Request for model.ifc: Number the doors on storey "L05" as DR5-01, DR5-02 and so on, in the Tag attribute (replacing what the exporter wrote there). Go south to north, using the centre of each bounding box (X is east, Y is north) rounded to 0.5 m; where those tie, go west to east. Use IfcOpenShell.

First a look at what the model holds.

```python
import ifcopenshell
import ifcopenshell.util.element
import ifcopenshell.util.placement

model = ifcopenshell.open("model.ifc")
print(model.schema)
storey = next(s for s in model.by_type("IfcBuildingStorey") if s.Name == "L05")
doors = [e for e in ifcopenshell.util.element.get_decomposition(storey) if e.is_a("IfcDoor")]
for e in sorted(doors, key=lambda e: e.id()):
    origin = ifcopenshell.util.placement.get_local_placement(e.ObjectPlacement)[:3, 3]
    print(e.id(), e.Tag, e.Name, origin.round(2) + 0.0, sep=" | ")
```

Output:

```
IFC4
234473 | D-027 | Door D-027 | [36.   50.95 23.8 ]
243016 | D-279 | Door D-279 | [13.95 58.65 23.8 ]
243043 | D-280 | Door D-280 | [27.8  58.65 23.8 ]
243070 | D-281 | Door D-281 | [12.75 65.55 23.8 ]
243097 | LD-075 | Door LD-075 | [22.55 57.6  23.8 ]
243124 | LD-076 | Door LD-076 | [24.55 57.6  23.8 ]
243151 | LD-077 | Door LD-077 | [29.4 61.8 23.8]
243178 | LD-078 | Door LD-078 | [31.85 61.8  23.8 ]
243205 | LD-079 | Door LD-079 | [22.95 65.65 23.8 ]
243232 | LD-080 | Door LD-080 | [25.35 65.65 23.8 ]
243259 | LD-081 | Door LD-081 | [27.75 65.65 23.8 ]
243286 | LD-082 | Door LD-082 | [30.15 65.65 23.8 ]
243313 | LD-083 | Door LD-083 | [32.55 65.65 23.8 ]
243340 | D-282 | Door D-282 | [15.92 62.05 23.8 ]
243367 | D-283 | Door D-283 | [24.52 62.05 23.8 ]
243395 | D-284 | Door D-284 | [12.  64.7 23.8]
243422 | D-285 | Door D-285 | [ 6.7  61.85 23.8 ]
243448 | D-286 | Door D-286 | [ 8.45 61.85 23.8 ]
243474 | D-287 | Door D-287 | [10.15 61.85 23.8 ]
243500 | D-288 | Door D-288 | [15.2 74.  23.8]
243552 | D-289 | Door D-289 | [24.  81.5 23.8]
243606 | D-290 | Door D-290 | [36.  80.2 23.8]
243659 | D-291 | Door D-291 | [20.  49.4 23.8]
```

```python
import ifcopenshell
import ifcopenshell.geom
import ifcopenshell.util.element
import ifcopenshell.util.shape

model = ifcopenshell.open("model.ifc")
settings = ifcopenshell.geom.settings()
settings.set("use-world-coords", True)


def centre(element):
    shape = ifcopenshell.geom.create_shape(settings, element)
    return ifcopenshell.util.shape.get_bbox_centroid(shape.geometry)


storey = next(s for s in model.by_type("IfcBuildingStorey") if s.Name == "L05")
doors = [e for e in ifcopenshell.util.element.get_decomposition(storey) if e.is_a("IfcDoor")]

# Insertion points can sit at a corner or the storey origin, so sort by the geometry (in metres).
centres = {e: centre(e) for e in doors}
doors.sort(key=lambda e: (round(centres[e][1] / 0.5), centres[e][0]))

for i, e in enumerate(doors, start=1):
    number = f"DR5-{i:02d}"
    e.Tag = number
    print(e.id(), number)

model.write("model_updated.ifc")
```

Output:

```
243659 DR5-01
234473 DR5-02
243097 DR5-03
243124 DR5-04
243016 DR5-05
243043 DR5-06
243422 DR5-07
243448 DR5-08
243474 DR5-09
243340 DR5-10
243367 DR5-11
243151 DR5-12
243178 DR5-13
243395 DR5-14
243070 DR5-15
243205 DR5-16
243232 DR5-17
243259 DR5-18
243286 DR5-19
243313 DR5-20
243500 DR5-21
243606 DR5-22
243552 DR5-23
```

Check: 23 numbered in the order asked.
